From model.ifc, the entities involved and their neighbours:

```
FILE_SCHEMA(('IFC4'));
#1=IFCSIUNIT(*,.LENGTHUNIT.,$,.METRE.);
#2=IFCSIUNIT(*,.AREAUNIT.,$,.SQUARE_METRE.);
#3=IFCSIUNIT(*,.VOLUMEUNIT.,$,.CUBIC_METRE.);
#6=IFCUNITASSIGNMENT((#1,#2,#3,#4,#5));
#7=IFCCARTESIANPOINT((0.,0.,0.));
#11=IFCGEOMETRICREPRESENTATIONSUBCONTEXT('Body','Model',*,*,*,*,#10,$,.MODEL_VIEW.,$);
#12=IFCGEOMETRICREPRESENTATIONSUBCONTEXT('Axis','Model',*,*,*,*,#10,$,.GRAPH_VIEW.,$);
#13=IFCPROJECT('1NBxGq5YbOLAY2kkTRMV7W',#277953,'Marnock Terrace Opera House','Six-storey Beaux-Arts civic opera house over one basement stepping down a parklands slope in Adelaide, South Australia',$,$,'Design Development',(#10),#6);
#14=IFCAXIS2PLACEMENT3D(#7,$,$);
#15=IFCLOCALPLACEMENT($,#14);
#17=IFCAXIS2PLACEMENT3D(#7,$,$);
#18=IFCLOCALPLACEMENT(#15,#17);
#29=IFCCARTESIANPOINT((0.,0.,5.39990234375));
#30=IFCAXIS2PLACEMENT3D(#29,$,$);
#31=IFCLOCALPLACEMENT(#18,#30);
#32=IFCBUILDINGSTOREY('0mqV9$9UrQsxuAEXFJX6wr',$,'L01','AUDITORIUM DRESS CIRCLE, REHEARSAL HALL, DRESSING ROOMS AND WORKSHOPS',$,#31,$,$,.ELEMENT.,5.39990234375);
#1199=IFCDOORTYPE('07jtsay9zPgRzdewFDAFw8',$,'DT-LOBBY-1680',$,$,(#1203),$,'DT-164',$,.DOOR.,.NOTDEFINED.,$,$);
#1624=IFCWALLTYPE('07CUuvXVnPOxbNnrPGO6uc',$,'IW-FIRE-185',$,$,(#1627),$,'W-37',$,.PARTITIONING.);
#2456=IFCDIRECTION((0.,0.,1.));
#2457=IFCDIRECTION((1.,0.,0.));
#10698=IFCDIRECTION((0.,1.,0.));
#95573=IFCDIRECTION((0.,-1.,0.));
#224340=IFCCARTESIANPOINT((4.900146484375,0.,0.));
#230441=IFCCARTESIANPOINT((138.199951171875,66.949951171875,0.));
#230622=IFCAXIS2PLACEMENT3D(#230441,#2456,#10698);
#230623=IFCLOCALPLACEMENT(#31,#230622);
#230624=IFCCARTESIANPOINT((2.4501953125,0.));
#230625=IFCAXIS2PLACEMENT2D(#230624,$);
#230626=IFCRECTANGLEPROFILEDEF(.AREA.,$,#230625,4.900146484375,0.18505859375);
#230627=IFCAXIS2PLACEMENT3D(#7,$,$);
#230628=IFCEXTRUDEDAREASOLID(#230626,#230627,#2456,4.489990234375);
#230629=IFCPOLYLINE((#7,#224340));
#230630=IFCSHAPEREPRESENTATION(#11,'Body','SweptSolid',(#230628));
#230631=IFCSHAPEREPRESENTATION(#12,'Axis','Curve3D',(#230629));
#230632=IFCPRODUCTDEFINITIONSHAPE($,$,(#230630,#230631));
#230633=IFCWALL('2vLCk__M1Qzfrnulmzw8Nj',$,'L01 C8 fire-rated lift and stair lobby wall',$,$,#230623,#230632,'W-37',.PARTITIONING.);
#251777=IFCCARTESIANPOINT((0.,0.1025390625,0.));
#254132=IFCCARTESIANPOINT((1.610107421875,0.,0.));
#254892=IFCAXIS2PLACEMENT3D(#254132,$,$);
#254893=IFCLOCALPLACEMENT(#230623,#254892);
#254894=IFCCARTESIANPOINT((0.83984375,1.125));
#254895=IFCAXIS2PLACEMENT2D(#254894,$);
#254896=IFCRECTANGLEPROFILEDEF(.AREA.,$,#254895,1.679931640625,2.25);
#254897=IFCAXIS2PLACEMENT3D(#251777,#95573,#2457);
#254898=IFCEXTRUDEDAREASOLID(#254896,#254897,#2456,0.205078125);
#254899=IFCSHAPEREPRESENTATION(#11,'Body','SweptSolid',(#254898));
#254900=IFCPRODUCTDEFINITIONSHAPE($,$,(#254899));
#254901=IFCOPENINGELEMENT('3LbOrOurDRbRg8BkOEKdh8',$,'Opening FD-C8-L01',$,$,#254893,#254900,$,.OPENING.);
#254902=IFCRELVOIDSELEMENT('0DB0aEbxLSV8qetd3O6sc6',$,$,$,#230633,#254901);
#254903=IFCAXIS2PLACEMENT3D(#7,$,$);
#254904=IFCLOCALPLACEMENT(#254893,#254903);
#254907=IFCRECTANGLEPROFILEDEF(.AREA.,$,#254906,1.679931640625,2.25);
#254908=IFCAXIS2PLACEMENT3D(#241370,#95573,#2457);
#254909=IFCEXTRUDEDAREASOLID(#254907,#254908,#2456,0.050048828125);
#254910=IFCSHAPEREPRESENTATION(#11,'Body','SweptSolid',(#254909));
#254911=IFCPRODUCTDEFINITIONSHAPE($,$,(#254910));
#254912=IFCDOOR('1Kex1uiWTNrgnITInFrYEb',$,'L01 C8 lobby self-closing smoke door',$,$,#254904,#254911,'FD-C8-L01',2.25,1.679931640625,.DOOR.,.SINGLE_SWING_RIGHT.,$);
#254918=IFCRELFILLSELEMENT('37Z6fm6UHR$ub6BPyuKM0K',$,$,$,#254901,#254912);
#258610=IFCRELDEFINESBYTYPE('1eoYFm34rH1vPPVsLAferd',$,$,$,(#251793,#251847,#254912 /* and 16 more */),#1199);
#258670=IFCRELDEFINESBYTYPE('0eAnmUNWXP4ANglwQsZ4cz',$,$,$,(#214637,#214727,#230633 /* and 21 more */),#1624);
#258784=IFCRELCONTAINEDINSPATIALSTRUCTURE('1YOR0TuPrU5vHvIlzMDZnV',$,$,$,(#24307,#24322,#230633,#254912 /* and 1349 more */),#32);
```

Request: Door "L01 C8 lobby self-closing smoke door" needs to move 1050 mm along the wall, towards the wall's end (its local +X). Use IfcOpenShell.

```python
import ifcopenshell
import ifcopenshell.api.geometry
import ifcopenshell.util.placement
import ifcopenshell.util.unit

model = ifcopenshell.open("model.ifc")
unit_scale = ifcopenshell.util.unit.calculate_unit_scale(model)

door = model.by_guid("1Kex1uiWTNrgnITInFrYEb")
opening = door.FillsVoids[0].RelatingOpeningElement
wall = opening.VoidsElements[0].RelatingBuildingElement

wall_matrix = ifcopenshell.util.placement.get_local_placement(wall.ObjectPlacement)
shift = wall_matrix[:3, 0] * 1.05 / unit_scale
before = ifcopenshell.util.placement.get_local_placement(door.ObjectPlacement)[:3, 3].copy()

# The door is placed relative to its opening, so it follows when the opening moves.
matrix = ifcopenshell.util.placement.get_local_placement(opening.ObjectPlacement)
matrix[:3, 3] += shift
ifcopenshell.api.geometry.edit_object_placement(
    model, product=opening, matrix=matrix, is_si=False, should_transform_children=True
)

after = ifcopenshell.util.placement.get_local_placement(door.ObjectPlacement)[:3, 3]
print("door moved by", (after - before).round(3) + 0.0)

model.write("model_updated.ifc")
```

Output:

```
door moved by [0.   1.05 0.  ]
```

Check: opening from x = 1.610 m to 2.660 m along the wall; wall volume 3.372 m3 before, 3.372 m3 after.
